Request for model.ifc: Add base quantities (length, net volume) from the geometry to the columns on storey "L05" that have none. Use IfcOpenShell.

First a look at what the model holds.

```python
import ifcopenshell
import ifcopenshell.util.element
import ifcopenshell.util.unit

model = ifcopenshell.open("model.ifc")
print(model.schema)
for unit_type in ("LENGTHUNIT", "AREAUNIT", "VOLUMEUNIT"):
    print(unit_type, ifcopenshell.util.unit.calculate_unit_scale(model, unit_type))
storey = next(s for s in model.by_type("IfcBuildingStorey") if s.Name == "L05")
columns = [e for e in ifcopenshell.util.element.get_decomposition(storey) if e.is_a("IfcColumn")]
for e in sorted(columns, key=lambda e: e.id()):
    print(e.id(), e.is_a(), e.Name, list(ifcopenshell.util.element.get_psets(e, qtos_only=True)), sep=" | ")
```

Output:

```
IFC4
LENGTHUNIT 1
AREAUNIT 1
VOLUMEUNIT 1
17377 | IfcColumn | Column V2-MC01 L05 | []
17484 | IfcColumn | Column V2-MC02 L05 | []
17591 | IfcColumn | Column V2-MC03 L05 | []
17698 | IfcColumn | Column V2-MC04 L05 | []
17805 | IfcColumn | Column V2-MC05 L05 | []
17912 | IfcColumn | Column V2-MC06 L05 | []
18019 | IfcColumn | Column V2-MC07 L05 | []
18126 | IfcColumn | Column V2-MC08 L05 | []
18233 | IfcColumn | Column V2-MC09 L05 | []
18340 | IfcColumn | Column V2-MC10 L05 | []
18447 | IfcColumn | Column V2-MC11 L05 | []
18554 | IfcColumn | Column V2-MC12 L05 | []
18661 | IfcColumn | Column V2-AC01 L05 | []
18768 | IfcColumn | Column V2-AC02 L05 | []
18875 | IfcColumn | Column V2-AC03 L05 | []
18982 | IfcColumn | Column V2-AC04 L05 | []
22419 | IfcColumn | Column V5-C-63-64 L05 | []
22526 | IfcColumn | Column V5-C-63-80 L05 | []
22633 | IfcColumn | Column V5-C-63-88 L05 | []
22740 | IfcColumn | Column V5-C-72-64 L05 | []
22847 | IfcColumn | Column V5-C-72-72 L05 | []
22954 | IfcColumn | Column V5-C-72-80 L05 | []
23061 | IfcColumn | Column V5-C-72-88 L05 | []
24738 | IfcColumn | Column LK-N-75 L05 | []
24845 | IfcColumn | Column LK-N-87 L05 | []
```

```python
import ifcopenshell
import ifcopenshell.api.pset
import ifcopenshell.geom
import ifcopenshell.util.element
import ifcopenshell.util.shape
import ifcopenshell.util.unit

model = ifcopenshell.open("model.ifc")
unit_scale = ifcopenshell.util.unit.calculate_unit_scale(model)
volume_scale = ifcopenshell.util.unit.calculate_unit_scale(model, "VOLUMEUNIT")
settings = ifcopenshell.geom.settings()

storey = next(s for s in model.by_type("IfcBuildingStorey") if s.Name == "L05")
columns = [e for e in ifcopenshell.util.element.get_decomposition(storey) if e.is_a("IfcColumn")]

for e in sorted(columns, key=lambda e: e.id()):
    if ifcopenshell.util.element.get_psets(e, qtos_only=True, should_inherit=False):
        continue
    # Geometry comes back in metres, in the element's own axes.
    shape = ifcopenshell.geom.create_shape(settings, e)
    values = {
        "Length": ifcopenshell.util.shape.get_z(shape.geometry) / unit_scale,
        "NetVolume": ifcopenshell.util.shape.get_volume(shape.geometry) / volume_scale,
    }
    qto = ifcopenshell.api.pset.add_qto(model, product=e, name="Qto_ColumnBaseQuantities")
    ifcopenshell.api.pset.edit_qto(model, qto=qto, properties=values)
    print(e.id(), {k: round(v, 3) for k, v in values.items()})

model.write("model_edited.ifc")
```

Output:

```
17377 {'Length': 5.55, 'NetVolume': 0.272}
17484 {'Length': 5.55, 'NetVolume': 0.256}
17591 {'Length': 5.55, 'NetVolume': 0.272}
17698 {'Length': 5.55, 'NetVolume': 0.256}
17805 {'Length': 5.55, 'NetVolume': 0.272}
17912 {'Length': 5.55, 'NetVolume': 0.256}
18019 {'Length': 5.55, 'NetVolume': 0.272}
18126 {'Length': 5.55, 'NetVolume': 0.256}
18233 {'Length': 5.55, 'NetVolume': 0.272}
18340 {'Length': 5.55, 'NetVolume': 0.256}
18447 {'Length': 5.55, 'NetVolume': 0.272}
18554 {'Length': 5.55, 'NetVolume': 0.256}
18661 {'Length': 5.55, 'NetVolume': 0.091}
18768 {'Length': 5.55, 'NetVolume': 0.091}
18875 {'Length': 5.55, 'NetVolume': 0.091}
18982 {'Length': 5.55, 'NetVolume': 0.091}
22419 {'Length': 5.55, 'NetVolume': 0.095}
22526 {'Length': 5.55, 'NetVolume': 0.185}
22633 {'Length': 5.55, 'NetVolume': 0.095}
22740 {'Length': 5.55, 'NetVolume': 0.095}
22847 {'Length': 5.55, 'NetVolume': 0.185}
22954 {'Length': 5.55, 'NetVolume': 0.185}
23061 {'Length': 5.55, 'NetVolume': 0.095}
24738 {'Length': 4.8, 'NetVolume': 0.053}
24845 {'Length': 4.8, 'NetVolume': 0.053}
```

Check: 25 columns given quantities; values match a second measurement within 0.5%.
